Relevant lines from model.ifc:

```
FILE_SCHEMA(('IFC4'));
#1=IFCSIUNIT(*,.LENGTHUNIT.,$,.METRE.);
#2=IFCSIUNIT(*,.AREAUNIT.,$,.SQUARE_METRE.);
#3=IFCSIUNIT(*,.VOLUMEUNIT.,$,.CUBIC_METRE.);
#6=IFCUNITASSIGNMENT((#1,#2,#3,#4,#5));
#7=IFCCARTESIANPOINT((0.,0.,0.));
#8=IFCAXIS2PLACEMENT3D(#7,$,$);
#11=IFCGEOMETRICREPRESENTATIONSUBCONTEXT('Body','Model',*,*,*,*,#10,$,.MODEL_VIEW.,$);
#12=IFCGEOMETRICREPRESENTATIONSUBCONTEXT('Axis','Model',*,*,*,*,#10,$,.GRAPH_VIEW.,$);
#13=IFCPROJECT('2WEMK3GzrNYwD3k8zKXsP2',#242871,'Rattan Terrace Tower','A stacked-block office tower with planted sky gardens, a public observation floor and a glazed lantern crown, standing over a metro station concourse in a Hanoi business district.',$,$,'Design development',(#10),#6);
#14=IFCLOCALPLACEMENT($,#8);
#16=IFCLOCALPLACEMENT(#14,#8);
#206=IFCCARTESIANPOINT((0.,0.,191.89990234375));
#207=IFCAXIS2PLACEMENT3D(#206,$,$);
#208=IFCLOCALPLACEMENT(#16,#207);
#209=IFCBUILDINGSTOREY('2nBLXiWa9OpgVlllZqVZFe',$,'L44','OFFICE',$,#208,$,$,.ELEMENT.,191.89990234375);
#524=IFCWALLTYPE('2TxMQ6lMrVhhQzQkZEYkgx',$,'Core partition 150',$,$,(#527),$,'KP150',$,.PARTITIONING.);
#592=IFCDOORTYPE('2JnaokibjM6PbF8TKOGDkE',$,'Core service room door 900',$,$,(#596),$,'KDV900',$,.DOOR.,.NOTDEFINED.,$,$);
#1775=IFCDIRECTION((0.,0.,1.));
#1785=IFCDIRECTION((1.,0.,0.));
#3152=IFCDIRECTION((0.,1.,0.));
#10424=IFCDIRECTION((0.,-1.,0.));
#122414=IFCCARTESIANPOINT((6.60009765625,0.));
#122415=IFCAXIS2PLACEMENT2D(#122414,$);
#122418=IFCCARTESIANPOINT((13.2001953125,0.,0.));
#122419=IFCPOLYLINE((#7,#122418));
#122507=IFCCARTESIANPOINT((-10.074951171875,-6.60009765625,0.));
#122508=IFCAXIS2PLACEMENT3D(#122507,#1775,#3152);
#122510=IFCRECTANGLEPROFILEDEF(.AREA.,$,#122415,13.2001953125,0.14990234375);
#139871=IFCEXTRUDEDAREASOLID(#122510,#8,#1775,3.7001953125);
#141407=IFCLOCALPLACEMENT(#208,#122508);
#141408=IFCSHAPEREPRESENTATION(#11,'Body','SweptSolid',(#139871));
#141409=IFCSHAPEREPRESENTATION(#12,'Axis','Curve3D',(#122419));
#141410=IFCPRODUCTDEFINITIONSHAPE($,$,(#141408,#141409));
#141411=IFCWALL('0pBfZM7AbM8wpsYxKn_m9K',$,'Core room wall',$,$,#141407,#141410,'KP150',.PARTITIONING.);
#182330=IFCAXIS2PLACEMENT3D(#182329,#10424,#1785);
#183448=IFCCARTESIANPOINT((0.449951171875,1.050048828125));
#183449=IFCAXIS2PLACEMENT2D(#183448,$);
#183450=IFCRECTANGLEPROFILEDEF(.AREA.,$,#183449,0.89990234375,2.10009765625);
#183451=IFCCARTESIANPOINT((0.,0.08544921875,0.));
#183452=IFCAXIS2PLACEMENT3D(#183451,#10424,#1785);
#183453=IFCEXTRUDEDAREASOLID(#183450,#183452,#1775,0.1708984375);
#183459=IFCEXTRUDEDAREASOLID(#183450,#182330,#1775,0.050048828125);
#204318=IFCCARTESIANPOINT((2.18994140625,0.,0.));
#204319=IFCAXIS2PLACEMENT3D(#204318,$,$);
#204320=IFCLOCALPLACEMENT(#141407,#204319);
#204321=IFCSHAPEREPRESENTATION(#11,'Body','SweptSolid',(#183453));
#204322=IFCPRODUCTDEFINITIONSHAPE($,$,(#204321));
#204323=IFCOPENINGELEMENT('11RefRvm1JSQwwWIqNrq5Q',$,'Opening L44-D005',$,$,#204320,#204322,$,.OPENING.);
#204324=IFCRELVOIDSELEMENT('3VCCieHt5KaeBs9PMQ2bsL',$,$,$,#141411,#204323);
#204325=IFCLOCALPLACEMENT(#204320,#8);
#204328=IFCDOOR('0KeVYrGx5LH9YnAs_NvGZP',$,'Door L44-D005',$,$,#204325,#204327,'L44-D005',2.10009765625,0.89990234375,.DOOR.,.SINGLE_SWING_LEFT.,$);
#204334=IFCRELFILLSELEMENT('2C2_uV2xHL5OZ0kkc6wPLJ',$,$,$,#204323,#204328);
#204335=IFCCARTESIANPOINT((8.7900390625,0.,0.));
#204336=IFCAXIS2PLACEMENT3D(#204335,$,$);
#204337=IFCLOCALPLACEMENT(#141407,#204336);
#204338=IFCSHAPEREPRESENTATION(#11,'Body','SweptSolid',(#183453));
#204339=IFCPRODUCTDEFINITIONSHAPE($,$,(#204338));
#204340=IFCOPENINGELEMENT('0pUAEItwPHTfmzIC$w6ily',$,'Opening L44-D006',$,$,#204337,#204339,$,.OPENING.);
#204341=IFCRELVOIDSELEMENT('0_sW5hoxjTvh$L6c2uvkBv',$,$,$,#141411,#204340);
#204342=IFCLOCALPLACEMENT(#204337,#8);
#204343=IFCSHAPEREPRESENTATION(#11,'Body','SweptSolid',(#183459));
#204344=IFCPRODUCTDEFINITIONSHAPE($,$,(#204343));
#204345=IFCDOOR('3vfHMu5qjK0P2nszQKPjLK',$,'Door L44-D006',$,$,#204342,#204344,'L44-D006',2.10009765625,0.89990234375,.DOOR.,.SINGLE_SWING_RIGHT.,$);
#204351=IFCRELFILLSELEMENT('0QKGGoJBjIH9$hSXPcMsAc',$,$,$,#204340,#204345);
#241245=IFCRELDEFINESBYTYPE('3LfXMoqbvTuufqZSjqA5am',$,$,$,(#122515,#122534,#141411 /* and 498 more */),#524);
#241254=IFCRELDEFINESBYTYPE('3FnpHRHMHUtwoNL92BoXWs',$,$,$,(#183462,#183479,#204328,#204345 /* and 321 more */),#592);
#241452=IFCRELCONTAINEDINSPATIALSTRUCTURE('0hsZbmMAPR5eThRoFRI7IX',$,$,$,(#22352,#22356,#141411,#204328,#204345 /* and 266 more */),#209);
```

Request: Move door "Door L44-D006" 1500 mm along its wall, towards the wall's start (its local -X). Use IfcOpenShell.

```python
import ifcopenshell
import ifcopenshell.api.geometry
import ifcopenshell.util.placement
import ifcopenshell.util.unit

model = ifcopenshell.open("model.ifc")
unit_scale = ifcopenshell.util.unit.calculate_unit_scale(model)

door = model.by_guid("3vfHMu5qjK0P2nszQKPjLK")
opening = door.FillsVoids[0].RelatingOpeningElement
wall = opening.VoidsElements[0].RelatingBuildingElement

wall_matrix = ifcopenshell.util.placement.get_local_placement(wall.ObjectPlacement)
shift = wall_matrix[:3, 0] * -1.5 / unit_scale
before = ifcopenshell.util.placement.get_local_placement(door.ObjectPlacement)[:3, 3].copy()

# The door is placed relative to its opening, so it follows when the opening moves.
matrix = ifcopenshell.util.placement.get_local_placement(opening.ObjectPlacement)
matrix[:3, 3] += shift
ifcopenshell.api.geometry.edit_object_placement(
    model, product=opening, matrix=matrix, is_si=False, should_transform_children=True
)

after = ifcopenshell.util.placement.get_local_placement(door.ObjectPlacement)[:3, 3]
print("door moved by", (after - before).round(3) + 0.0)

model.write("model_rev.ifc")
```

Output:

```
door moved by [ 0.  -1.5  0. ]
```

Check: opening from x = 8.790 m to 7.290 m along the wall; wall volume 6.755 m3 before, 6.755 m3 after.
